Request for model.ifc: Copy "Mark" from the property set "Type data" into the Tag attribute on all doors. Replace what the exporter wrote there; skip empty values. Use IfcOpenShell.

First a look at what the model holds.

```python
import ifcopenshell
import ifcopenshell.util.element

model = ifcopenshell.open("model.ifc")
print(model.schema)
doors = model.by_type("IfcDoor")
print(len(doors), "doors")
for e in doors[:8]:
    source = ifcopenshell.util.element.get_pset(e, "Type data", "Mark")
    target = e.Tag
    print(e.id(), repr(source), repr(target), sep=" | ")
```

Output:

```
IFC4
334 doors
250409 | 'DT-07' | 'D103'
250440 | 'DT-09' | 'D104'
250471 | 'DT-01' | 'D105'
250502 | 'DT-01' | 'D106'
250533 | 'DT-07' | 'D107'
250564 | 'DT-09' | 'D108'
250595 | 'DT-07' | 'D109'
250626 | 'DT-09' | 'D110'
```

```python
import ifcopenshell
import ifcopenshell.util.element

model = ifcopenshell.open("model.ifc")

count = 0
for e in model.by_type("IfcDoor"):
    value = ifcopenshell.util.element.get_pset(e, "Type data", "Mark")
    current = e.Tag
    if not value or not value.strip() or current == value:
        continue
    e.Tag = value
    count += 1

print(count, "doors updated")

model.write("model_updated.ifc")
```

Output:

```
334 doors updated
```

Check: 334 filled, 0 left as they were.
